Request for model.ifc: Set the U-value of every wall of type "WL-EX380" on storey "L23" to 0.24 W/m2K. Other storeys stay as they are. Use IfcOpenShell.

First a look at what the model holds.

```python
import ifcopenshell
import ifcopenshell.util.element

model = ifcopenshell.open("model.ifc")
print(model.schema)
storey = next(s for s in model.by_type("IfcBuildingStorey") if s.Name == "L23")
walls = [e for e in ifcopenshell.util.element.get_decomposition(storey) if e.is_a("IfcWall")]
seen = {}
for e in walls:
    element_type = ifcopenshell.util.element.get_type(e)
    key = (element_type.Name if element_type != e and element_type else None, ifcopenshell.util.element.get_pset(e, "Pset_WallCommon", "ThermalTransmittance"))
    seen[key] = seen.get(key, 0) + 1
for (name, value), count in sorted(seen.items(), key=str):
    print(count, "x", name, "|", value)
```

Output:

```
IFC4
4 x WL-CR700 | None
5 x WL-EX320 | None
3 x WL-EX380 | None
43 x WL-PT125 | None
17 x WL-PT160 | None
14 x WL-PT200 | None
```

```python
import ifcopenshell
import ifcopenshell.api.pset
import ifcopenshell.util.element

model = ifcopenshell.open("model.ifc")

storey = next(s for s in model.by_type("IfcBuildingStorey") if s.Name == "L23")
walls = [e for e in ifcopenshell.util.element.get_decomposition(storey) if e.is_a("IfcWall")]

count = 0
for e in walls:
    element_type = ifcopenshell.util.element.get_type(e)
    if element_type in (None, e) or element_type.Name != "WL-EX380":
        continue
    # add_pset returns the element's existing set when there is one.
    pset = ifcopenshell.api.pset.add_pset(model, product=e, name="Pset_WallCommon")
    ifcopenshell.api.pset.edit_pset(model, pset=pset, properties={"ThermalTransmittance": 0.24})
    count += 1

print(count, "walls updated")

model.write("model_edited.ifc")
```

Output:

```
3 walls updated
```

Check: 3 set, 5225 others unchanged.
